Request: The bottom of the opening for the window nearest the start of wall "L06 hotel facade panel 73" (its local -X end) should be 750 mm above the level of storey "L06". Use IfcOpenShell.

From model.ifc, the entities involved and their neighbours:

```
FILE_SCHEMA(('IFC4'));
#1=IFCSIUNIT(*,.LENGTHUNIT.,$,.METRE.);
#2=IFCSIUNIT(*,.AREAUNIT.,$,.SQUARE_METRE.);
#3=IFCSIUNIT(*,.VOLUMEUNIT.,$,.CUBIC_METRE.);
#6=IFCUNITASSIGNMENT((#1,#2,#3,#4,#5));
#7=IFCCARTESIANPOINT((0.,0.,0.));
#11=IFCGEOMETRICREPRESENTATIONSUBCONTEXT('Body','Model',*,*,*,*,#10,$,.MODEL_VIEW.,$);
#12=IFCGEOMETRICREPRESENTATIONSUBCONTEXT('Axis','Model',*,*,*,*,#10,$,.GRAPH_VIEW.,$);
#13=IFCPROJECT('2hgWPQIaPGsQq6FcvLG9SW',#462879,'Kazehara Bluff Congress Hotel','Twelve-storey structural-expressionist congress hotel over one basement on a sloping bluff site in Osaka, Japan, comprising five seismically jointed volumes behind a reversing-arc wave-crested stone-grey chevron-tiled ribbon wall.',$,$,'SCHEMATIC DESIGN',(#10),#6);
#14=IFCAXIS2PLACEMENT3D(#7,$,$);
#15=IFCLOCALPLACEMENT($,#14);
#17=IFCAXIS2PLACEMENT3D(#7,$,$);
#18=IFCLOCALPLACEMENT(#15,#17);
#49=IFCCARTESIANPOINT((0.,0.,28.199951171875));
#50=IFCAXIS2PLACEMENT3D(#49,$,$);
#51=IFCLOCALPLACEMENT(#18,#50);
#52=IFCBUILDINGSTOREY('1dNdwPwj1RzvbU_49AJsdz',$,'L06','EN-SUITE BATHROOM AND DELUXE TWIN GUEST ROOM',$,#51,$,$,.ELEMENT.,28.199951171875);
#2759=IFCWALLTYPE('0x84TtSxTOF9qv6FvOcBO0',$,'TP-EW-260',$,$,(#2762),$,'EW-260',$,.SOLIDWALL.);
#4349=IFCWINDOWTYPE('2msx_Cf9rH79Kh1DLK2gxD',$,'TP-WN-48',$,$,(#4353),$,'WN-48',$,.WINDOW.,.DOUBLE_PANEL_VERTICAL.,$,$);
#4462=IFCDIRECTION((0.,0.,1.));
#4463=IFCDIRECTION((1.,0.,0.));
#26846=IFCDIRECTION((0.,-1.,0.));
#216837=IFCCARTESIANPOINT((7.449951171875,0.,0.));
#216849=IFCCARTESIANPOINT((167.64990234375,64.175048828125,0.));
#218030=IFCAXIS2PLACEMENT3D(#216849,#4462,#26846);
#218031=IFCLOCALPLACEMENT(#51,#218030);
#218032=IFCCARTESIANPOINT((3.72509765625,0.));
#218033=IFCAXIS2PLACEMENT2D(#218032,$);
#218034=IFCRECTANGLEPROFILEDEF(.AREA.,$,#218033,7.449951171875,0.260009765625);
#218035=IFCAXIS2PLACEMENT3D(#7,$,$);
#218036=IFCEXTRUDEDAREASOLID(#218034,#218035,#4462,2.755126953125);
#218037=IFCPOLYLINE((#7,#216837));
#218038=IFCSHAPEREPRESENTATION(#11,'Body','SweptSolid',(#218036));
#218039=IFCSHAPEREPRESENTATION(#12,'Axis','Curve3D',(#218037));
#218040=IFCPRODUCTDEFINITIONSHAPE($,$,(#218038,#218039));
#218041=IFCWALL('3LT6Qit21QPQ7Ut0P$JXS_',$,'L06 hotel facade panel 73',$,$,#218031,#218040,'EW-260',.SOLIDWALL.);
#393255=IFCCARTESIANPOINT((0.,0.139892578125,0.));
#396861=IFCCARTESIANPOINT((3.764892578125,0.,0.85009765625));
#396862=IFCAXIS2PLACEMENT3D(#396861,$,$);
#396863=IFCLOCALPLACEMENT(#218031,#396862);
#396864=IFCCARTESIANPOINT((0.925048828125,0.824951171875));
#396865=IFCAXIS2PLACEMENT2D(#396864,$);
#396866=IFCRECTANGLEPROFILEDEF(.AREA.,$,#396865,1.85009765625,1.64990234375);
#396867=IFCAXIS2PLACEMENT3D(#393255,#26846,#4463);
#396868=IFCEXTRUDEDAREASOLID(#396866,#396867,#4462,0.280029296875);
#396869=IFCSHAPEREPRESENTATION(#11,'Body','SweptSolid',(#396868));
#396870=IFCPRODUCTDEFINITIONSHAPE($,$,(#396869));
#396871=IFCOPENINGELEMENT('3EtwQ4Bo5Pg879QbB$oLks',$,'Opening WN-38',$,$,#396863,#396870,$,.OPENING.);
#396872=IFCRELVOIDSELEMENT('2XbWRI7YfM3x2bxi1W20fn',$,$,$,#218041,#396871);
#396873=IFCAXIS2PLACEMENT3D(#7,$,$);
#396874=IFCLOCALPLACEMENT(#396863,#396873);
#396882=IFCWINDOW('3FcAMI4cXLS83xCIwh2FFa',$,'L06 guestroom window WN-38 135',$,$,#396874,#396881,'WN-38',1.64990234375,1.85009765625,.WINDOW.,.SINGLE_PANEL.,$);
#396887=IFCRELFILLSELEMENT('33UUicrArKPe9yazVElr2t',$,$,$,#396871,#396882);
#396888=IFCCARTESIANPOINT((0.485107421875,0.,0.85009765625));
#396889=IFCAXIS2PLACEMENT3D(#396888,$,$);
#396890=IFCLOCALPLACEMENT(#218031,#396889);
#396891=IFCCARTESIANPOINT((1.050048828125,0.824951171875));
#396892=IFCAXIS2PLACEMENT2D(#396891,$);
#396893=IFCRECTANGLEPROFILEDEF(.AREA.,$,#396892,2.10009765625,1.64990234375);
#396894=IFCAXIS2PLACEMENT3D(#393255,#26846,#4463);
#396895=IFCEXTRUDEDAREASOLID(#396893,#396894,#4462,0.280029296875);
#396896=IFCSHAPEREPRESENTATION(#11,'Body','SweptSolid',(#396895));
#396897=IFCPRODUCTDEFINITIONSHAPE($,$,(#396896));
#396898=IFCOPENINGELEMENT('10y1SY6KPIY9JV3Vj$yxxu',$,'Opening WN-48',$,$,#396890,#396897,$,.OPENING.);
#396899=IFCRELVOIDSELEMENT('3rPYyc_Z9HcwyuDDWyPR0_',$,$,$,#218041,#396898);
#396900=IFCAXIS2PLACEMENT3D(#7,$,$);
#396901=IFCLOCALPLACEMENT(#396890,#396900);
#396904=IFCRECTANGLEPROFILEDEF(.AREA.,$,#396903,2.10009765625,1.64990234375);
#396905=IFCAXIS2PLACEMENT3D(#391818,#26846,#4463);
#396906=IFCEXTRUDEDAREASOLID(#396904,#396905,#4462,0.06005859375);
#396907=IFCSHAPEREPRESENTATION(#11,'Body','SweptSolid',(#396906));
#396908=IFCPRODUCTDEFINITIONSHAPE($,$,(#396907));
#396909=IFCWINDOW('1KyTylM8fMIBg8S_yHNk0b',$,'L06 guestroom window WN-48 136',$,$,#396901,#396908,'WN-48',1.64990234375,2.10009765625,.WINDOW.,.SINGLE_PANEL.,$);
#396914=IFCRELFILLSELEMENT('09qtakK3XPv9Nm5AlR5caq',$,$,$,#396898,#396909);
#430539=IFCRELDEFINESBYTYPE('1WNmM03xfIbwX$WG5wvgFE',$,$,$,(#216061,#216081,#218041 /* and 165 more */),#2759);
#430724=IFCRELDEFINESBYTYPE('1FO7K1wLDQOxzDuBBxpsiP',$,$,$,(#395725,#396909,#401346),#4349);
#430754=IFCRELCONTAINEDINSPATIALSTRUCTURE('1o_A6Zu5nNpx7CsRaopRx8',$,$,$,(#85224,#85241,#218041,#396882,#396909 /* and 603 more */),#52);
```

```python
import numpy as np
import ifcopenshell
import ifcopenshell.api.geometry
import ifcopenshell.geom
import ifcopenshell.util.element
import ifcopenshell.util.placement
import ifcopenshell.util.shape
import ifcopenshell.util.unit

model = ifcopenshell.open("model.ifc")
unit_scale = ifcopenshell.util.unit.calculate_unit_scale(model)

window = model.by_guid("1KyTylM8fMIBg8S_yHNk0b")
opening = window.FillsVoids[0].RelatingOpeningElement
storey = ifcopenshell.util.element.get_container(window, ifc_class="IfcBuildingStorey")
level = ifcopenshell.util.placement.get_local_placement(storey.ObjectPlacement)[2, 3]

# The opening's origin need not be at the sill, so measure its lowest point.
shape = ifcopenshell.geom.create_shape(ifcopenshell.geom.settings(), opening)
bottom = ifcopenshell.util.shape.get_shape_bottom_elevation(shape, shape.geometry) / unit_scale
dz = level + 0.75 - bottom

shift = np.array([0.0, 0.0, dz])
# The window is placed relative to its opening, so it follows when the opening moves.
matrix = ifcopenshell.util.placement.get_local_placement(opening.ObjectPlacement)
matrix[:3, 3] += shift
ifcopenshell.api.geometry.edit_object_placement(
    model, product=opening, matrix=matrix, is_si=False, should_transform_children=True
)

print(f"moved by {dz * unit_scale:+.3f} m")

model.write("model_v2.ifc")
```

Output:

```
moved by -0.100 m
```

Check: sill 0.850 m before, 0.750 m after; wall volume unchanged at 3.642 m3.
